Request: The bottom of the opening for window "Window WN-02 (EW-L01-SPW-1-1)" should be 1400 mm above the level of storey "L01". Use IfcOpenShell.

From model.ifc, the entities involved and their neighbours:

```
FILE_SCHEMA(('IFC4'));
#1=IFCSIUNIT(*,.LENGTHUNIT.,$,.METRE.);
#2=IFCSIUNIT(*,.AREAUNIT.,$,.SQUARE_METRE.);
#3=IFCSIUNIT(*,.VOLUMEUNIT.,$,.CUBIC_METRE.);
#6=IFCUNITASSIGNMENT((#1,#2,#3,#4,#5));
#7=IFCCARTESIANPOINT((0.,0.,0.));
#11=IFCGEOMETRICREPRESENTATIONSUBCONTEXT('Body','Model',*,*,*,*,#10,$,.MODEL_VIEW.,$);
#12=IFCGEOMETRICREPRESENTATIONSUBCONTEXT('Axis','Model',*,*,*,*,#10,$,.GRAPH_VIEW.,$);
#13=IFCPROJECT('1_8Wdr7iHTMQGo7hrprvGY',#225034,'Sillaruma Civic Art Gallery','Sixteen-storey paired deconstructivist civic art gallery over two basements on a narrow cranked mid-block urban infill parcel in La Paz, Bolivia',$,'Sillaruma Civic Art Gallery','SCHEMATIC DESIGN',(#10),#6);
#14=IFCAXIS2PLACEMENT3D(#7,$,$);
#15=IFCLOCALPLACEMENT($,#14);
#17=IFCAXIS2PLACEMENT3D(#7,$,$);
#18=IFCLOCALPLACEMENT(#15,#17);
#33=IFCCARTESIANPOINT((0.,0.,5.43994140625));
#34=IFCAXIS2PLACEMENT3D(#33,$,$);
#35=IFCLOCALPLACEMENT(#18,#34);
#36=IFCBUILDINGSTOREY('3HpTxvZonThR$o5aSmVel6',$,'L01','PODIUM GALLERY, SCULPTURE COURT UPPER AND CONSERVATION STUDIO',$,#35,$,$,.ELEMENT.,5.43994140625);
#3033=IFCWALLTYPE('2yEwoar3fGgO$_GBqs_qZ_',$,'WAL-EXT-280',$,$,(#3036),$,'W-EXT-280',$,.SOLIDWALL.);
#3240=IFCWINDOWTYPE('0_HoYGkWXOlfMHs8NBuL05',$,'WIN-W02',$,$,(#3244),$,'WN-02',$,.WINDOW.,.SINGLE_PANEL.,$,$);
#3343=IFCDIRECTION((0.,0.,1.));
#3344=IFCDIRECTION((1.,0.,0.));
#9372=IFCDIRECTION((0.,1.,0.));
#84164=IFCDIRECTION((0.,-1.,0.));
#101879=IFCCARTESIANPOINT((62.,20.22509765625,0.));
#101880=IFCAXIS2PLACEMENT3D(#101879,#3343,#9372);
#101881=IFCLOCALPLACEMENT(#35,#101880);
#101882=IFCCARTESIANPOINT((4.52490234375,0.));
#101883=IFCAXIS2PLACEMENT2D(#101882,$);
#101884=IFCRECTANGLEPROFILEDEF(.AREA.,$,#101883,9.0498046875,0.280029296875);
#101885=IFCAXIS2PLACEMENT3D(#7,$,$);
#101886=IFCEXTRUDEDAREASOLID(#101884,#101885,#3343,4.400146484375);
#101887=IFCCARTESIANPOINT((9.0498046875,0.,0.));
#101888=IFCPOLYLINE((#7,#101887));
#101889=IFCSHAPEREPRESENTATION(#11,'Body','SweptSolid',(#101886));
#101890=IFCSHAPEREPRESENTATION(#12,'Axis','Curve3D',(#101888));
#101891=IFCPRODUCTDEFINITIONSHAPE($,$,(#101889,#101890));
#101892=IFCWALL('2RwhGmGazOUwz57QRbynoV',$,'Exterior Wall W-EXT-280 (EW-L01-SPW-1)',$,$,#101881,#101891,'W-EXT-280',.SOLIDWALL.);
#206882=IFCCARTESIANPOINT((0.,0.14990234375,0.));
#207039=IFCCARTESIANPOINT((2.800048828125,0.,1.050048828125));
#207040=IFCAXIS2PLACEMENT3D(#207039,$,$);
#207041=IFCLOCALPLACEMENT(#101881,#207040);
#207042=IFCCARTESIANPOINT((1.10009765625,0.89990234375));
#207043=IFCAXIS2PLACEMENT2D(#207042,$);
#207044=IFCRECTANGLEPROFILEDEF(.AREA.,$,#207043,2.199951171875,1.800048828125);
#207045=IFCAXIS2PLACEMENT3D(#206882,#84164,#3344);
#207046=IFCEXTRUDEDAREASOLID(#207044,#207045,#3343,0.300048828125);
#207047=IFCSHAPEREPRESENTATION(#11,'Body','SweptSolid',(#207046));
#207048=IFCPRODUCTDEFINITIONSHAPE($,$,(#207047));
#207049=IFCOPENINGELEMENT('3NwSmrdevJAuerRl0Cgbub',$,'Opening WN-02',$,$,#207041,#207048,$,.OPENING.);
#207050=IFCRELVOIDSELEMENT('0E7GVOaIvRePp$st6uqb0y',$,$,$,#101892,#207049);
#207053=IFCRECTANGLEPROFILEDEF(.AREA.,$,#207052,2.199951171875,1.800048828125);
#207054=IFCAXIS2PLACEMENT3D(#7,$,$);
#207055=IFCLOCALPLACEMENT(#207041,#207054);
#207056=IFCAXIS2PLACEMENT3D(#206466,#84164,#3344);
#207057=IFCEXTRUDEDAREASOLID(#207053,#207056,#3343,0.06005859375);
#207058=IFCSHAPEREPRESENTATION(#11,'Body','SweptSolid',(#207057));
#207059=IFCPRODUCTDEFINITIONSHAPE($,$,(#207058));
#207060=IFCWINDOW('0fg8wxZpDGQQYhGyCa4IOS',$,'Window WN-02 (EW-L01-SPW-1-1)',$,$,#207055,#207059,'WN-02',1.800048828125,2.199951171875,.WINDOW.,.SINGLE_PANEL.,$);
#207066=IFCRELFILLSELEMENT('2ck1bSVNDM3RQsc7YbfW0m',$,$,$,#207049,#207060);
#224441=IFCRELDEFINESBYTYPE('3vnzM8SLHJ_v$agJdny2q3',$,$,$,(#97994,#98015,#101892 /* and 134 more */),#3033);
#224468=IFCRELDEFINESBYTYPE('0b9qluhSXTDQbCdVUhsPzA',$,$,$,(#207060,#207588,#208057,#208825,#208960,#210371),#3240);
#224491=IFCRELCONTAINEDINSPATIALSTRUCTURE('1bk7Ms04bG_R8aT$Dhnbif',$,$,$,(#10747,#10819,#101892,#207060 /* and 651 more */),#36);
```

```python
import numpy as np
import ifcopenshell
import ifcopenshell.api.geometry
import ifcopenshell.geom
import ifcopenshell.util.element
import ifcopenshell.util.placement
import ifcopenshell.util.shape
import ifcopenshell.util.unit

model = ifcopenshell.open("model.ifc")
unit_scale = ifcopenshell.util.unit.calculate_unit_scale(model)

window = model.by_guid("0fg8wxZpDGQQYhGyCa4IOS")
opening = window.FillsVoids[0].RelatingOpeningElement
storey = ifcopenshell.util.element.get_container(window, ifc_class="IfcBuildingStorey")
level = ifcopenshell.util.placement.get_local_placement(storey.ObjectPlacement)[2, 3]

# The opening's origin need not be at the sill, so measure its lowest point.
shape = ifcopenshell.geom.create_shape(ifcopenshell.geom.settings(), opening)
bottom = ifcopenshell.util.shape.get_shape_bottom_elevation(shape, shape.geometry) / unit_scale
dz = level + 1.4 - bottom

shift = np.array([0.0, 0.0, dz])
# The window is placed relative to its opening, so it follows when the opening moves.
matrix = ifcopenshell.util.placement.get_local_placement(opening.ObjectPlacement)
matrix[:3, 3] += shift
ifcopenshell.api.geometry.edit_object_placement(
    model, product=opening, matrix=matrix, is_si=False, should_transform_children=True
)

print(f"moved by {dz * unit_scale:+.3f} m")

model.write("model_updated.ifc")
```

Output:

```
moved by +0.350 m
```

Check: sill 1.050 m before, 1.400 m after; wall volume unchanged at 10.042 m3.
